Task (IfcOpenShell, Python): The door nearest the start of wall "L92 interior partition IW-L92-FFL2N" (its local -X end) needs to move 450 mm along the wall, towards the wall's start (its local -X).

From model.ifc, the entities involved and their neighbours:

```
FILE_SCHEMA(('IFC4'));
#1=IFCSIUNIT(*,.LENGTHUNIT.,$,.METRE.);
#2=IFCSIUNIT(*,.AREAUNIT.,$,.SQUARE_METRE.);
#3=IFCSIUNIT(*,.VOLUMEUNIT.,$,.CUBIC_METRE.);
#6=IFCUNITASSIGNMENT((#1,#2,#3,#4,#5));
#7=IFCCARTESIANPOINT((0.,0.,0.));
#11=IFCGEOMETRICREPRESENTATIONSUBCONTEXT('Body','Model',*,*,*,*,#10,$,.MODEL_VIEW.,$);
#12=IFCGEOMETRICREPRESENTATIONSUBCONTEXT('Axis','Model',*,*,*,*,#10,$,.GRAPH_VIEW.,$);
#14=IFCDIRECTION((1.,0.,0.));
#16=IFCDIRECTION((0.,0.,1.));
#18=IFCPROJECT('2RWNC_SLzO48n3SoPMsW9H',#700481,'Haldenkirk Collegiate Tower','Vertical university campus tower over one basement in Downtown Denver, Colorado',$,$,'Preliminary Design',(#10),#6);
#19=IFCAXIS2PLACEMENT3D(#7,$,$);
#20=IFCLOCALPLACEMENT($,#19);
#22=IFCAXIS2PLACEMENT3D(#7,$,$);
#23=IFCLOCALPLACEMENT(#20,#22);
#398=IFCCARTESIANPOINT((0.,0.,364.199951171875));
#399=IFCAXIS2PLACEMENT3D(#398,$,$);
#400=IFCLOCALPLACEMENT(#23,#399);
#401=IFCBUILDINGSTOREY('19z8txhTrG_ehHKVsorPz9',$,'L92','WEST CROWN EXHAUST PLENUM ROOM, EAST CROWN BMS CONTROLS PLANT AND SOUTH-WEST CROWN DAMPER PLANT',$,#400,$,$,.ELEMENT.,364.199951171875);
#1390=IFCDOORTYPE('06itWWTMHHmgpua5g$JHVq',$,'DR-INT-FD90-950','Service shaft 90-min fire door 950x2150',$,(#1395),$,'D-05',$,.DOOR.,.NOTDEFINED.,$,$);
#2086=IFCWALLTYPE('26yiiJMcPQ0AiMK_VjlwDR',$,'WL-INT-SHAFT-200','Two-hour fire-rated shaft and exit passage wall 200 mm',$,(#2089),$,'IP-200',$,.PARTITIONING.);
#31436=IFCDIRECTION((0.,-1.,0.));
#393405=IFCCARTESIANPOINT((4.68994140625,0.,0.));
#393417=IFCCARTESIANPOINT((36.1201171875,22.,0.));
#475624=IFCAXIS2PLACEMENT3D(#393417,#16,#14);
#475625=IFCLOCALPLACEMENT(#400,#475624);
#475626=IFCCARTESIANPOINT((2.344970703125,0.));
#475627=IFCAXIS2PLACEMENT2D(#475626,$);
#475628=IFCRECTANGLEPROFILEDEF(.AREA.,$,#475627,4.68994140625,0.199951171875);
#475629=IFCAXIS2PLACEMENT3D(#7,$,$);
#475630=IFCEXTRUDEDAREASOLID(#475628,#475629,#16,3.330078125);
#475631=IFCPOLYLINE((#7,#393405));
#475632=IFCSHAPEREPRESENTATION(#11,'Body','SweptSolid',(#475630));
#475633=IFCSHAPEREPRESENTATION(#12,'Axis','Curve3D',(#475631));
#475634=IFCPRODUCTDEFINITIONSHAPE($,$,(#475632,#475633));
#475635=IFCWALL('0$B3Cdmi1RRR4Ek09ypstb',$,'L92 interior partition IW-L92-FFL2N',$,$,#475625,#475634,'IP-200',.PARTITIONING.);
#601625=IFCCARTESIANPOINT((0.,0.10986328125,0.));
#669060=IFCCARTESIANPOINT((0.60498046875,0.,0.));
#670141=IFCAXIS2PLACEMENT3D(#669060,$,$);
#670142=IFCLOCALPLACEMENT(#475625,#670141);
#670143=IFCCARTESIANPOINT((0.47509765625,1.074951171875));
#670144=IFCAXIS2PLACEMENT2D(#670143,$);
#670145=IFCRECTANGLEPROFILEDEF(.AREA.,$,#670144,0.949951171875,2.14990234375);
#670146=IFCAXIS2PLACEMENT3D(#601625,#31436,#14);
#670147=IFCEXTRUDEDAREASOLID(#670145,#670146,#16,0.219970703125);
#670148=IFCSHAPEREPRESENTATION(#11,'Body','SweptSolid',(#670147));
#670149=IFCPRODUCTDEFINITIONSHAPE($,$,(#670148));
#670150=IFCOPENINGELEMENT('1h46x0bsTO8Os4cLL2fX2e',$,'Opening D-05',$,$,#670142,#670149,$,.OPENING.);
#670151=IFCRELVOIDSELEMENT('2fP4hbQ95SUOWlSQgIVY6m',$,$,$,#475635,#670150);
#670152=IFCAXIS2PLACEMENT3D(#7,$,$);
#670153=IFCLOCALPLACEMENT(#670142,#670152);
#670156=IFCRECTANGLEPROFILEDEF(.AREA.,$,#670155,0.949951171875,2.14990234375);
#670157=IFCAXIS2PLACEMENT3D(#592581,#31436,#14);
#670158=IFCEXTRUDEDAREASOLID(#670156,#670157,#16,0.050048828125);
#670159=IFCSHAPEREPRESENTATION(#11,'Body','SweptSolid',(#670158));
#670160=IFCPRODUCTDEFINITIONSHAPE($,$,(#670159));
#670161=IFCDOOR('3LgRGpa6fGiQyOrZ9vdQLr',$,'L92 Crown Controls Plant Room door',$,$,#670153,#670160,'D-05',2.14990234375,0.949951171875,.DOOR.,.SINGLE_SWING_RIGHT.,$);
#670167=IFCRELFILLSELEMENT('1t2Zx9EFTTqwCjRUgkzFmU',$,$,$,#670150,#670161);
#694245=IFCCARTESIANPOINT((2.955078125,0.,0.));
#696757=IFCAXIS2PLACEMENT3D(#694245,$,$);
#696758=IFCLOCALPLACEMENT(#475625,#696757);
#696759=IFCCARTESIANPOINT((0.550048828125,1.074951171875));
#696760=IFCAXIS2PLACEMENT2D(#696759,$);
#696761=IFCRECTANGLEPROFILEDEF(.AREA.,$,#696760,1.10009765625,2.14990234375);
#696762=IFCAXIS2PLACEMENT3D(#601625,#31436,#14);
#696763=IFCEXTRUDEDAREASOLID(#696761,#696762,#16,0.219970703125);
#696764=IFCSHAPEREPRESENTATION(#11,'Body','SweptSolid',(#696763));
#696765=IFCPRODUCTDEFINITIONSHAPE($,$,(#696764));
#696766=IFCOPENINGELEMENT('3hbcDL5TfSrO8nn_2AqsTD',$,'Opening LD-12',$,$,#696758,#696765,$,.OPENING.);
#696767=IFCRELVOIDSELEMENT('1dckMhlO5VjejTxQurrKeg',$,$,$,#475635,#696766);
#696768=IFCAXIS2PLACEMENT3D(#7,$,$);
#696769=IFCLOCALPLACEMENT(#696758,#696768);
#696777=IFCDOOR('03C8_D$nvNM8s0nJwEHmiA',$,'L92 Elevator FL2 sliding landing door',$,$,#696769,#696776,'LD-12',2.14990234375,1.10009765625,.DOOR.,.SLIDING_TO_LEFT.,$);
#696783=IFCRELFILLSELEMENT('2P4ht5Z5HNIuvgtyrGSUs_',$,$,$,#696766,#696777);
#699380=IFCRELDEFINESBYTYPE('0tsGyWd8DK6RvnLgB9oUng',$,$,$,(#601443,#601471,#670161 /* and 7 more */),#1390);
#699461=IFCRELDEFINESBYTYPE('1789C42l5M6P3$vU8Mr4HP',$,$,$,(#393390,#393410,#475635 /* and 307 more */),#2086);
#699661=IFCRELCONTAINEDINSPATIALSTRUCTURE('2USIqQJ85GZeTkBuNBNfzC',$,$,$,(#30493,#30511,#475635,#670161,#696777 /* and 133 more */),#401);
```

```python
import ifcopenshell
import ifcopenshell.api.geometry
import ifcopenshell.util.placement
import ifcopenshell.util.unit

model = ifcopenshell.open("model.ifc")
unit_scale = ifcopenshell.util.unit.calculate_unit_scale(model)

door = model.by_id(670161)
opening = door.FillsVoids[0].RelatingOpeningElement
wall = opening.VoidsElements[0].RelatingBuildingElement

wall_matrix = ifcopenshell.util.placement.get_local_placement(wall.ObjectPlacement)
shift = wall_matrix[:3, 0] * -0.45 / unit_scale
before = ifcopenshell.util.placement.get_local_placement(door.ObjectPlacement)[:3, 3].copy()

# The door is placed relative to its opening, so it follows when the opening moves.
matrix = ifcopenshell.util.placement.get_local_placement(opening.ObjectPlacement)
matrix[:3, 3] += shift
ifcopenshell.api.geometry.edit_object_placement(
    model, product=opening, matrix=matrix, is_si=False, should_transform_children=True
)

after = ifcopenshell.util.placement.get_local_placement(door.ObjectPlacement)[:3, 3]
print("door moved by", (after - before).round(3) + 0.0)

model.write("model_rev.ifc")
```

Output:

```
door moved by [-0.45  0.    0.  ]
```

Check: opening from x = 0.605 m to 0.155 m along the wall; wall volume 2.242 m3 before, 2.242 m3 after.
